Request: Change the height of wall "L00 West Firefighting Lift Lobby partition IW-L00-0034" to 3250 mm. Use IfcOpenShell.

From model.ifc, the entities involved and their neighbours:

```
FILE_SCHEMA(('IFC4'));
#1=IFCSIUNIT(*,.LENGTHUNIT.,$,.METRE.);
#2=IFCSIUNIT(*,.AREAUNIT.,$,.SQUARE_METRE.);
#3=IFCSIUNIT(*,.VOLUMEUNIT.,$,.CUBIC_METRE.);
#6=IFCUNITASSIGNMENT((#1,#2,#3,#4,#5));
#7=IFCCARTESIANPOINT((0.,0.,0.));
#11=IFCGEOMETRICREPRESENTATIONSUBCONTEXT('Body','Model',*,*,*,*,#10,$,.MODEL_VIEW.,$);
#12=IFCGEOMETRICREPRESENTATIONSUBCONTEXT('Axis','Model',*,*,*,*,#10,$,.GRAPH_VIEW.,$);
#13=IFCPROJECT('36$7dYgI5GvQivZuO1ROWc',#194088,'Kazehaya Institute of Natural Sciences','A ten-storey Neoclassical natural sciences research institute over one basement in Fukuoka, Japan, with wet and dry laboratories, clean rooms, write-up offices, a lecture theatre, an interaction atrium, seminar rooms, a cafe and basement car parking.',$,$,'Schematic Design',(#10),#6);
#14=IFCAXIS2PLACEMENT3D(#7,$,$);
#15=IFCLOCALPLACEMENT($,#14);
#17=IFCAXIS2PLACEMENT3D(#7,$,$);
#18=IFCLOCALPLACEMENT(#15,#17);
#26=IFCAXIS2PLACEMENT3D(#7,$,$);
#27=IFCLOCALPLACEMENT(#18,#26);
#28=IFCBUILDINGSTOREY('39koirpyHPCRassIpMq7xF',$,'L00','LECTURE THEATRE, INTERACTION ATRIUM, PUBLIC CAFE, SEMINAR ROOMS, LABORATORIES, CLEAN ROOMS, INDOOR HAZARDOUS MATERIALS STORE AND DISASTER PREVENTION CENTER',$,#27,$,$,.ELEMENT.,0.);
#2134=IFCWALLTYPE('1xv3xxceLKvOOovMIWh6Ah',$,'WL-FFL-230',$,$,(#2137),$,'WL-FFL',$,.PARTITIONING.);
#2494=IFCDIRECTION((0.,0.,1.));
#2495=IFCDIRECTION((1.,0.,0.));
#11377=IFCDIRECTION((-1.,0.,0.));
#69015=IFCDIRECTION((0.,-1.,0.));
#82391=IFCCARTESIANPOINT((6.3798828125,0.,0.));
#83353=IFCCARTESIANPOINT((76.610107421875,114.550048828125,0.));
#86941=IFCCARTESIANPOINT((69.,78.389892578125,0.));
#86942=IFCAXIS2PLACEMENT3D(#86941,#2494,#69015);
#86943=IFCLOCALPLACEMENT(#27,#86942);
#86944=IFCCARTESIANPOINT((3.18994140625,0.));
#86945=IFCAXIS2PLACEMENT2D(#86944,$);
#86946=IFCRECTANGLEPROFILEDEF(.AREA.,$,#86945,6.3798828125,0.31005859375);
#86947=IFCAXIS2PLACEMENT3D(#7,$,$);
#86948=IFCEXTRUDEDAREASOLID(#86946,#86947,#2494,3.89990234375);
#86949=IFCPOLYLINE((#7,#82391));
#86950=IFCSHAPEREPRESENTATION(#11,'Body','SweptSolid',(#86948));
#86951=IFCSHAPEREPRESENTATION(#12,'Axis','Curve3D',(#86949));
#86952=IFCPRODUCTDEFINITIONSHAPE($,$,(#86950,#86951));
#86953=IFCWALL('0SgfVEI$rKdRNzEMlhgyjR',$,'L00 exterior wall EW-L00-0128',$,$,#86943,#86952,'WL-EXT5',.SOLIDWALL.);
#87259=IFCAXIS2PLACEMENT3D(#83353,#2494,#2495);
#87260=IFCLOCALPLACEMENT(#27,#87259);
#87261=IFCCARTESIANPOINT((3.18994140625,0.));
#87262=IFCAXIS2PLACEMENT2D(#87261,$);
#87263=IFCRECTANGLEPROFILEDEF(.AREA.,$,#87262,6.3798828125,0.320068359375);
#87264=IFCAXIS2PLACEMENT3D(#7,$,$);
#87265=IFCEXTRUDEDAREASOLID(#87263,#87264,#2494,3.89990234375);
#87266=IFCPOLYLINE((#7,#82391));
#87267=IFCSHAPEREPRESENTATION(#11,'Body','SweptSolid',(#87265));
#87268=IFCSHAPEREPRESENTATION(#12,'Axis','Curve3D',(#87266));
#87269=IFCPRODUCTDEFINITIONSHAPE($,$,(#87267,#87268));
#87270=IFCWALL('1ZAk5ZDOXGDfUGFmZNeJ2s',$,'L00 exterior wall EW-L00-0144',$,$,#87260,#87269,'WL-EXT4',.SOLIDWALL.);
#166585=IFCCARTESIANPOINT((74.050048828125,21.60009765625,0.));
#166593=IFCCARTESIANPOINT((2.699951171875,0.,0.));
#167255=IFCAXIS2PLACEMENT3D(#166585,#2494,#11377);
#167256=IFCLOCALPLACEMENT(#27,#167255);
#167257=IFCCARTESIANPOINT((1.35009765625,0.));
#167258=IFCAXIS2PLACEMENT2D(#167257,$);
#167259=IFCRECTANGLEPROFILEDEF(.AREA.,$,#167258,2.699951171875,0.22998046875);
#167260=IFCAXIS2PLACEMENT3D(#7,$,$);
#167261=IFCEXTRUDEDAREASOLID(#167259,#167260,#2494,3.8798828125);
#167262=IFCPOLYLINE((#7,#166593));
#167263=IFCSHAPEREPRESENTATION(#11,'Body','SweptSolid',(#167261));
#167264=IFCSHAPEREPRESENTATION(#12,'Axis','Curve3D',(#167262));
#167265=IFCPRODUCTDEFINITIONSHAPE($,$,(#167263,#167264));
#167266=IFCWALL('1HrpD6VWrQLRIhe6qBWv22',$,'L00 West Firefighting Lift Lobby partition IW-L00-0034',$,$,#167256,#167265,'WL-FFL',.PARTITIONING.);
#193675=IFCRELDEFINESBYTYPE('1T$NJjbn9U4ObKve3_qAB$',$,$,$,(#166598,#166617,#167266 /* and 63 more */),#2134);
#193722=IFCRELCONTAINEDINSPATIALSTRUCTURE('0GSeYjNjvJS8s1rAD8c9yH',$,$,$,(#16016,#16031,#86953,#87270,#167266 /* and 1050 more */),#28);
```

```python
import ifcopenshell
import ifcopenshell.geom
import ifcopenshell.util.representation
import ifcopenshell.util.shape
import ifcopenshell.util.unit

model = ifcopenshell.open("model.ifc")
unit_scale = ifcopenshell.util.unit.calculate_unit_scale(model)
settings = ifcopenshell.geom.settings()


def volume(element):
    """Net volume in cubic metres, openings subtracted."""
    shape = ifcopenshell.geom.create_shape(settings, element)
    return ifcopenshell.util.shape.get_volume(shape.geometry)


wall = model.by_guid("1HrpD6VWrQLRIhe6qBWv22")
before = volume(wall)

body = ifcopenshell.util.representation.get_representation(wall, "Model", "Body")
solid = body.Items[0]
old_height = solid.Depth
solid.Depth = 3.25 / unit_scale
after = volume(wall)

print(f"height {old_height:g} -> {solid.Depth:g}, volume {before:.3f} -> {after:.3f} m3")

model.write("model_v2.ifc")
```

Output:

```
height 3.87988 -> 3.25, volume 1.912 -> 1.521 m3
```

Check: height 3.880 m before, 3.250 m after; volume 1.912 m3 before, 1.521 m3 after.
